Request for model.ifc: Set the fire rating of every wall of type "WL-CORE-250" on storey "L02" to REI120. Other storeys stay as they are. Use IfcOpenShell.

First a look at what the model holds.

```python
import ifcopenshell
import ifcopenshell.util.element

model = ifcopenshell.open("model.ifc")
print(model.schema)
storey = next(s for s in model.by_type("IfcBuildingStorey") if s.Name == "L02")
walls = [e for e in ifcopenshell.util.element.get_decomposition(storey) if e.is_a("IfcWall")]
seen = {}
for e in walls:
    element_type = ifcopenshell.util.element.get_type(e)
    key = (element_type.Name if element_type != e and element_type else None, ifcopenshell.util.element.get_pset(e, "Pset_WallCommon", "FireRating"))
    seen[key] = seen.get(key, 0) + 1
for (name, value), count in sorted(seen.items(), key=str):
    print(count, "x", name, "|", value)
```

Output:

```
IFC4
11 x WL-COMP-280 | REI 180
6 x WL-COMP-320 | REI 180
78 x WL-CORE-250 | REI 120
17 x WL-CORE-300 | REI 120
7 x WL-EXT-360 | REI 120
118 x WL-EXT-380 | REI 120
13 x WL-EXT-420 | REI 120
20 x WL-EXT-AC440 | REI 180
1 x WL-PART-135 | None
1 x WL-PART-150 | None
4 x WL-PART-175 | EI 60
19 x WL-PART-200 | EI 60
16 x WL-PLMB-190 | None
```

```python
import ifcopenshell
import ifcopenshell.api.pset
import ifcopenshell.util.element

model = ifcopenshell.open("model.ifc")

storey = next(s for s in model.by_type("IfcBuildingStorey") if s.Name == "L02")
walls = [e for e in ifcopenshell.util.element.get_decomposition(storey) if e.is_a("IfcWall")]

count = 0
for e in walls:
    element_type = ifcopenshell.util.element.get_type(e)
    if element_type in (None, e) or element_type.Name != "WL-CORE-250":
        continue
    # add_pset returns the element's existing set when there is one.
    pset = ifcopenshell.api.pset.add_pset(model, product=e, name="Pset_WallCommon")
    ifcopenshell.api.pset.edit_pset(model, pset=pset, properties={"FireRating": "REI120"})
    count += 1

print(count, "walls updated")

model.write("model_updated.ifc")
```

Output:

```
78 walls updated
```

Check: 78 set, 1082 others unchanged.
